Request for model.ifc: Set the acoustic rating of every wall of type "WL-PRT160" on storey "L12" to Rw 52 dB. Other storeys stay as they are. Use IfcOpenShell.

First a look at what the model holds.

```python
import ifcopenshell
import ifcopenshell.util.element

model = ifcopenshell.open("model.ifc")
print(model.schema)
storey = next(s for s in model.by_type("IfcBuildingStorey") if s.Name == "L12")
walls = [e for e in ifcopenshell.util.element.get_decomposition(storey) if e.is_a("IfcWall")]
seen = {}
for e in walls:
    element_type = ifcopenshell.util.element.get_type(e)
    key = (element_type.Name if element_type != e and element_type else None, ifcopenshell.util.element.get_pset(e, "Pset_WallCommon", "AcousticRating"))
    seen[key] = seen.get(key, 0) + 1
for (name, value), count in sorted(seen.items(), key=str):
    print(count, "x", name, "|", value)
```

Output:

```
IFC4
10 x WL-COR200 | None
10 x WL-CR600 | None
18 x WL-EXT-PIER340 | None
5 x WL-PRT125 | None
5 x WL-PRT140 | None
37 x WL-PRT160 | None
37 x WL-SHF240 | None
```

```python
import ifcopenshell
import ifcopenshell.api.pset
import ifcopenshell.util.element

model = ifcopenshell.open("model.ifc")

storey = next(s for s in model.by_type("IfcBuildingStorey") if s.Name == "L12")
walls = [e for e in ifcopenshell.util.element.get_decomposition(storey) if e.is_a("IfcWall")]

count = 0
for e in walls:
    element_type = ifcopenshell.util.element.get_type(e)
    if element_type in (None, e) or element_type.Name != "WL-PRT160":
        continue
    found = ifcopenshell.util.element.get_pset(e, "Pset_WallCommon", should_inherit=False)
    if found:
        pset = model.by_id(found["id"])
        if len(ifcopenshell.util.element.get_elements_by_pset(pset)) > 1:
            pset = ifcopenshell.api.pset.unshare_pset(model, products=[e], pset=pset)[0]
    else:
        pset = ifcopenshell.api.pset.add_pset(model, product=e, name="Pset_WallCommon")
    ifcopenshell.api.pset.edit_pset(model, pset=pset, properties={"AcousticRating": "Rw 52 dB"})
    count += 1

print(count, "walls updated")

model.write("model_rev.ifc")
```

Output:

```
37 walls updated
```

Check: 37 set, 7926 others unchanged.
